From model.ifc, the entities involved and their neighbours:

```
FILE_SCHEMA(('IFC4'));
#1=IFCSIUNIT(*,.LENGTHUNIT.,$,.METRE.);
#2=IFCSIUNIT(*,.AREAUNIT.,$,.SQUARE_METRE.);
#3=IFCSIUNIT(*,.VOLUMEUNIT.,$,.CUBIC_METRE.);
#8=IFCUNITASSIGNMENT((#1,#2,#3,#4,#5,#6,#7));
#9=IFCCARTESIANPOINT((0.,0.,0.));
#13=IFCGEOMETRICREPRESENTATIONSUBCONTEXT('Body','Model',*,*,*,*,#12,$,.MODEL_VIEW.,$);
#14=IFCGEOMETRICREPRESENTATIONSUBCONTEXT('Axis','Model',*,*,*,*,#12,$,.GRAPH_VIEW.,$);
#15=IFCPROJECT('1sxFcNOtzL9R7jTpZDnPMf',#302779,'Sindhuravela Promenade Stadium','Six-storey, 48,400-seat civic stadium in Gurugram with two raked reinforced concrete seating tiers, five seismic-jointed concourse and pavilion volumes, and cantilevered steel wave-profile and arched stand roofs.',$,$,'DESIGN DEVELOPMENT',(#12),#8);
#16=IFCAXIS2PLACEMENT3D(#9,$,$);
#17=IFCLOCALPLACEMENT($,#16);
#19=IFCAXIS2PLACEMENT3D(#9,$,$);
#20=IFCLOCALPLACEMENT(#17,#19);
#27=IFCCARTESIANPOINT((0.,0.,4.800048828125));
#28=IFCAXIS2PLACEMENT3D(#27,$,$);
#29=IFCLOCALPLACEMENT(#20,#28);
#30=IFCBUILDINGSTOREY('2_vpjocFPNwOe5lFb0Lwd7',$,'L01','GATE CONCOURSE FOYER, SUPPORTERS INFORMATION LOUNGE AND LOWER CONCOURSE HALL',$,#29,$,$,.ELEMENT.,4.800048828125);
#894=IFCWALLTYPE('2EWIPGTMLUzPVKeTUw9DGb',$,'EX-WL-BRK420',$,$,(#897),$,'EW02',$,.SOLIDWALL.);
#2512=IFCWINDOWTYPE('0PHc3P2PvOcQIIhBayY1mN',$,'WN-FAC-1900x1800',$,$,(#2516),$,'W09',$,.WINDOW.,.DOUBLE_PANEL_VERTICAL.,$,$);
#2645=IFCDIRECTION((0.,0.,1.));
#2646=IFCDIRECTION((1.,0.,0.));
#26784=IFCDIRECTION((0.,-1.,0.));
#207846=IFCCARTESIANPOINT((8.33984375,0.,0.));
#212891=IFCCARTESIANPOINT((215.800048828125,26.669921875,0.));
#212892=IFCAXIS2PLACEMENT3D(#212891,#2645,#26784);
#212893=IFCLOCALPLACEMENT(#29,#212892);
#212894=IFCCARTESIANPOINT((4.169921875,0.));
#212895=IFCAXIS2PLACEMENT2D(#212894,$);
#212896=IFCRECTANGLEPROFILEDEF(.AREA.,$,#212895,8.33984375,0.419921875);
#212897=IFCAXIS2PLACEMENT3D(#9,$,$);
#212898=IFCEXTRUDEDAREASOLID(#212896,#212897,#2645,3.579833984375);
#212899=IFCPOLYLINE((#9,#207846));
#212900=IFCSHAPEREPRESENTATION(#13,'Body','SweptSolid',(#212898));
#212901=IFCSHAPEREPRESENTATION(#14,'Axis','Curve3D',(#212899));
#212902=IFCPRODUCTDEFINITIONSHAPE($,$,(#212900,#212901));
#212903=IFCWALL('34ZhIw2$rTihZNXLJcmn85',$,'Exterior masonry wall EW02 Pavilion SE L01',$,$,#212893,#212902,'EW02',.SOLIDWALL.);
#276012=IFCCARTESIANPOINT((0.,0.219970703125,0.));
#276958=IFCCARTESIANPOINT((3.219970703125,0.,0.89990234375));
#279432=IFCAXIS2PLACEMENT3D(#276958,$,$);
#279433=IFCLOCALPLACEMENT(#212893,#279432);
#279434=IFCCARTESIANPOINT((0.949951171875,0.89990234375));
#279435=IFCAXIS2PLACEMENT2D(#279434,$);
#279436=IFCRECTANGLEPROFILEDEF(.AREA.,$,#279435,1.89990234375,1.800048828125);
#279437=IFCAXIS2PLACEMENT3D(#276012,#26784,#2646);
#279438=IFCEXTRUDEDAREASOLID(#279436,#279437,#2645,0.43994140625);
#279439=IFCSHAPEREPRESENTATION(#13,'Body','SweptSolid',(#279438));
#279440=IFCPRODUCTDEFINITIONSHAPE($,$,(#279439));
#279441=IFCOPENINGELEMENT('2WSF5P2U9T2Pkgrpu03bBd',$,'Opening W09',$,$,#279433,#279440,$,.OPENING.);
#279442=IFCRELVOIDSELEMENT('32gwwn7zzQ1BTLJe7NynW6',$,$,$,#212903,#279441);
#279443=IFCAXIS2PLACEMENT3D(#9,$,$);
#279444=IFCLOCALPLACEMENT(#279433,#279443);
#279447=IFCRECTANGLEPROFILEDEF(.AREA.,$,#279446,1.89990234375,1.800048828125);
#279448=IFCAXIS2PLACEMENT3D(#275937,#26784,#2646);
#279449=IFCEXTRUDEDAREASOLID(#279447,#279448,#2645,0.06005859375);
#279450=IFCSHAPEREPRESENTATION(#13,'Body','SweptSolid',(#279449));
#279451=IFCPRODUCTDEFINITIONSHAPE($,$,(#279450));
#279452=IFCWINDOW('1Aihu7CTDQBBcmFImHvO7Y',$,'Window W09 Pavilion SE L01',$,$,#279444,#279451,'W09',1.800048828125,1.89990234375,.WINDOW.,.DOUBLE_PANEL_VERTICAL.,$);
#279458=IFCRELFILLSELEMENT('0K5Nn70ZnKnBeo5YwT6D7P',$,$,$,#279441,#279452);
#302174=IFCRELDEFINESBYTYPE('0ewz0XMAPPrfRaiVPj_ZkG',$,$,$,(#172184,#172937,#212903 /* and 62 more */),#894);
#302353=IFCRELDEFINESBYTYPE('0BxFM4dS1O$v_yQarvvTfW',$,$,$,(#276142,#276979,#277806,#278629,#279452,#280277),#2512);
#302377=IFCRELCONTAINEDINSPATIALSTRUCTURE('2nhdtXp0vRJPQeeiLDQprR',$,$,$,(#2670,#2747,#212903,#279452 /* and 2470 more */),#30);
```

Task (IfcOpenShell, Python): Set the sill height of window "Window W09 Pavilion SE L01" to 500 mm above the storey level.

```python
import numpy as np
import ifcopenshell
import ifcopenshell.api.geometry
import ifcopenshell.geom
import ifcopenshell.util.element
import ifcopenshell.util.placement
import ifcopenshell.util.shape
import ifcopenshell.util.unit

model = ifcopenshell.open("model.ifc")
unit_scale = ifcopenshell.util.unit.calculate_unit_scale(model)

window = model.by_guid("1Aihu7CTDQBBcmFImHvO7Y")
opening = window.FillsVoids[0].RelatingOpeningElement
storey = ifcopenshell.util.element.get_container(window, ifc_class="IfcBuildingStorey")
level = ifcopenshell.util.placement.get_local_placement(storey.ObjectPlacement)[2, 3]

# The opening's origin need not be at the sill, so measure its lowest point.
shape = ifcopenshell.geom.create_shape(ifcopenshell.geom.settings(), opening)
bottom = ifcopenshell.util.shape.get_shape_bottom_elevation(shape, shape.geometry) / unit_scale
dz = level + 0.5 / unit_scale - bottom

shift = np.array([0.0, 0.0, dz])
# The window is placed relative to its opening, so it follows when the opening moves.
matrix = ifcopenshell.util.placement.get_local_placement(opening.ObjectPlacement)
matrix[:3, 3] += shift
ifcopenshell.api.geometry.edit_object_placement(
    model, product=opening, matrix=matrix, is_si=False, should_transform_children=True
)

print(f"moved by {dz * unit_scale:+.3f} m")

model.write("model_updated.ifc")
```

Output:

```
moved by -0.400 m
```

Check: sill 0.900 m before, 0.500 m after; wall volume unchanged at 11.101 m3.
